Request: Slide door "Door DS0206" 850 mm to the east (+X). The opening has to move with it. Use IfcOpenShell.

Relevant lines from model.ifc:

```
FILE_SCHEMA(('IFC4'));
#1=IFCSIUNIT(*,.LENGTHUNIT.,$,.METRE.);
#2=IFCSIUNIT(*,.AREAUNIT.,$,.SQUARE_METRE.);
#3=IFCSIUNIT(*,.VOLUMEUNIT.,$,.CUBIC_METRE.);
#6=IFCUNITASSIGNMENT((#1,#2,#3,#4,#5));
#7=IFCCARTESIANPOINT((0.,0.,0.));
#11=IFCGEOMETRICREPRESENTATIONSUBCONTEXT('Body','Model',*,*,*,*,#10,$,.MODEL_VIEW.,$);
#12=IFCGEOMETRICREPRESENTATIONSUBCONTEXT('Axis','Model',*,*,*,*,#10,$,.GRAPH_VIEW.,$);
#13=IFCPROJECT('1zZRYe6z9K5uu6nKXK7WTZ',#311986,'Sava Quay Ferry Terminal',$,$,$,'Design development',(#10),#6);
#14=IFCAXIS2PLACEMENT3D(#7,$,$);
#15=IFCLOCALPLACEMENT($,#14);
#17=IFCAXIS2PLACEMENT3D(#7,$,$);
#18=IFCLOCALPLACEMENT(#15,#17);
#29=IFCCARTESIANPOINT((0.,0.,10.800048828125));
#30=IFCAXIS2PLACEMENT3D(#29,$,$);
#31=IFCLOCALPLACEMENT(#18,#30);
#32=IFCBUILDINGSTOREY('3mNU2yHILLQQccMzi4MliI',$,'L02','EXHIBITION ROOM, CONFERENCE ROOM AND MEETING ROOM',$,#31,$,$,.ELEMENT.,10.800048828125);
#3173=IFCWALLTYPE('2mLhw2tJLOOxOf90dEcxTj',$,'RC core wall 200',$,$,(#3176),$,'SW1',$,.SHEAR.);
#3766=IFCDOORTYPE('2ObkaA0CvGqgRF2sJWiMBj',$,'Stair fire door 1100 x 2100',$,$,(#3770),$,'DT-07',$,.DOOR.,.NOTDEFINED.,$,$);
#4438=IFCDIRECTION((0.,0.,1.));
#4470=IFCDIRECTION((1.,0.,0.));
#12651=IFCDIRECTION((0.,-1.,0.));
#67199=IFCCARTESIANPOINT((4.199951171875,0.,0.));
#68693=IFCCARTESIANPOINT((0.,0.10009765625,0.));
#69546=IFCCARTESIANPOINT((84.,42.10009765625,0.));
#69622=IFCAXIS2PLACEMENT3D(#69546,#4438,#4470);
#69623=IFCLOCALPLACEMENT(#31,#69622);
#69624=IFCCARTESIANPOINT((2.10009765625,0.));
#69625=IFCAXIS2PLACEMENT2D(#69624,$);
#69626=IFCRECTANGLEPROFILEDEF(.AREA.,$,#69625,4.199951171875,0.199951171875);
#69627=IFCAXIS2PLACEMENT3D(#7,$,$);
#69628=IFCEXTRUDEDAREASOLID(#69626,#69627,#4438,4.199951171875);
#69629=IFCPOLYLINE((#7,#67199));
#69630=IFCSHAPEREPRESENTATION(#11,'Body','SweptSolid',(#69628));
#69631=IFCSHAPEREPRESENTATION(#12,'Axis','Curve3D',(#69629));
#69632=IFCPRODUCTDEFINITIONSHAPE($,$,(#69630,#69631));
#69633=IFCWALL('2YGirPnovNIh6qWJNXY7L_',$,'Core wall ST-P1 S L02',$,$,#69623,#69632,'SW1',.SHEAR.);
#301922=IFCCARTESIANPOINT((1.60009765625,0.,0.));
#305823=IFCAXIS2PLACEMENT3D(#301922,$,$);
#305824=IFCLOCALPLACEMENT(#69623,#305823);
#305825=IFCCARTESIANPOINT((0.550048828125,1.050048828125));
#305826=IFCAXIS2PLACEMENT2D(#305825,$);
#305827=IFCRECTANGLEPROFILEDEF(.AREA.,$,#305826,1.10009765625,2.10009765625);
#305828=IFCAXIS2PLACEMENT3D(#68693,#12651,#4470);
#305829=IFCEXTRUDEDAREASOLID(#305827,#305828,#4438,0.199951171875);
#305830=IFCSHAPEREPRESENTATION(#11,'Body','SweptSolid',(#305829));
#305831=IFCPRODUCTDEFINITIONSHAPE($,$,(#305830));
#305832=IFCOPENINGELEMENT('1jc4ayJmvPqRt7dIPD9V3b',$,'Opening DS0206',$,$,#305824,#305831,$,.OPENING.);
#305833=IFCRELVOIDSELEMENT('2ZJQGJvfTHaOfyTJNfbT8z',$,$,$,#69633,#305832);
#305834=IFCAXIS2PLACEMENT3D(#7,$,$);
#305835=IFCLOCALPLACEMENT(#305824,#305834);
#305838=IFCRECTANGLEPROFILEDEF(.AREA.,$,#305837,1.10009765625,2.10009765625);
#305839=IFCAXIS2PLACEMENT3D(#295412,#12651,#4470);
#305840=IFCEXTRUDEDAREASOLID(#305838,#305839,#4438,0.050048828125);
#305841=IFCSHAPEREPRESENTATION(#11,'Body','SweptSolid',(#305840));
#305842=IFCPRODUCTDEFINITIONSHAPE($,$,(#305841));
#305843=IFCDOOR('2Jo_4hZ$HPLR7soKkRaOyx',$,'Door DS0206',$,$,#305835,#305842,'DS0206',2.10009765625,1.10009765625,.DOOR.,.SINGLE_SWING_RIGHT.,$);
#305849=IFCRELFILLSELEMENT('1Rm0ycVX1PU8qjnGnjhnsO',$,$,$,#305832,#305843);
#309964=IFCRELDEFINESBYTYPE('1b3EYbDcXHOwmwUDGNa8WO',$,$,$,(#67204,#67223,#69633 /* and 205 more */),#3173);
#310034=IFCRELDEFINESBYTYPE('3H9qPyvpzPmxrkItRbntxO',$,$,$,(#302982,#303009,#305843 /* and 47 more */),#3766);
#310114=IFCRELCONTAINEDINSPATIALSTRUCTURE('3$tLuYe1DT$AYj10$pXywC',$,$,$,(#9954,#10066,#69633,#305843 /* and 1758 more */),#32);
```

```python
import ifcopenshell
import ifcopenshell.api.geometry
import ifcopenshell.util.placement

model = ifcopenshell.open("model.ifc")

door = model.by_guid("2Jo_4hZ$HPLR7soKkRaOyx")
opening = door.FillsVoids[0].RelatingOpeningElement
wall = opening.VoidsElements[0].RelatingBuildingElement

wall_matrix = ifcopenshell.util.placement.get_local_placement(wall.ObjectPlacement)
shift = wall_matrix[:3, 0] * 0.85
before = ifcopenshell.util.placement.get_local_placement(door.ObjectPlacement)[:3, 3].copy()

# The door is placed relative to its opening, so it follows when the opening moves.
matrix = ifcopenshell.util.placement.get_local_placement(opening.ObjectPlacement)
matrix[:3, 3] += shift
ifcopenshell.api.geometry.edit_object_placement(
    model, product=opening, matrix=matrix, is_si=False, should_transform_children=True
)

after = ifcopenshell.util.placement.get_local_placement(door.ObjectPlacement)[:3, 3]
print("door moved by", (after - before).round(3) + 0.0)

model.write("model-out.ifc")
```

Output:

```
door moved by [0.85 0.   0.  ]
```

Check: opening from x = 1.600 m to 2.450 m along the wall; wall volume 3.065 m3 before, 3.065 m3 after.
